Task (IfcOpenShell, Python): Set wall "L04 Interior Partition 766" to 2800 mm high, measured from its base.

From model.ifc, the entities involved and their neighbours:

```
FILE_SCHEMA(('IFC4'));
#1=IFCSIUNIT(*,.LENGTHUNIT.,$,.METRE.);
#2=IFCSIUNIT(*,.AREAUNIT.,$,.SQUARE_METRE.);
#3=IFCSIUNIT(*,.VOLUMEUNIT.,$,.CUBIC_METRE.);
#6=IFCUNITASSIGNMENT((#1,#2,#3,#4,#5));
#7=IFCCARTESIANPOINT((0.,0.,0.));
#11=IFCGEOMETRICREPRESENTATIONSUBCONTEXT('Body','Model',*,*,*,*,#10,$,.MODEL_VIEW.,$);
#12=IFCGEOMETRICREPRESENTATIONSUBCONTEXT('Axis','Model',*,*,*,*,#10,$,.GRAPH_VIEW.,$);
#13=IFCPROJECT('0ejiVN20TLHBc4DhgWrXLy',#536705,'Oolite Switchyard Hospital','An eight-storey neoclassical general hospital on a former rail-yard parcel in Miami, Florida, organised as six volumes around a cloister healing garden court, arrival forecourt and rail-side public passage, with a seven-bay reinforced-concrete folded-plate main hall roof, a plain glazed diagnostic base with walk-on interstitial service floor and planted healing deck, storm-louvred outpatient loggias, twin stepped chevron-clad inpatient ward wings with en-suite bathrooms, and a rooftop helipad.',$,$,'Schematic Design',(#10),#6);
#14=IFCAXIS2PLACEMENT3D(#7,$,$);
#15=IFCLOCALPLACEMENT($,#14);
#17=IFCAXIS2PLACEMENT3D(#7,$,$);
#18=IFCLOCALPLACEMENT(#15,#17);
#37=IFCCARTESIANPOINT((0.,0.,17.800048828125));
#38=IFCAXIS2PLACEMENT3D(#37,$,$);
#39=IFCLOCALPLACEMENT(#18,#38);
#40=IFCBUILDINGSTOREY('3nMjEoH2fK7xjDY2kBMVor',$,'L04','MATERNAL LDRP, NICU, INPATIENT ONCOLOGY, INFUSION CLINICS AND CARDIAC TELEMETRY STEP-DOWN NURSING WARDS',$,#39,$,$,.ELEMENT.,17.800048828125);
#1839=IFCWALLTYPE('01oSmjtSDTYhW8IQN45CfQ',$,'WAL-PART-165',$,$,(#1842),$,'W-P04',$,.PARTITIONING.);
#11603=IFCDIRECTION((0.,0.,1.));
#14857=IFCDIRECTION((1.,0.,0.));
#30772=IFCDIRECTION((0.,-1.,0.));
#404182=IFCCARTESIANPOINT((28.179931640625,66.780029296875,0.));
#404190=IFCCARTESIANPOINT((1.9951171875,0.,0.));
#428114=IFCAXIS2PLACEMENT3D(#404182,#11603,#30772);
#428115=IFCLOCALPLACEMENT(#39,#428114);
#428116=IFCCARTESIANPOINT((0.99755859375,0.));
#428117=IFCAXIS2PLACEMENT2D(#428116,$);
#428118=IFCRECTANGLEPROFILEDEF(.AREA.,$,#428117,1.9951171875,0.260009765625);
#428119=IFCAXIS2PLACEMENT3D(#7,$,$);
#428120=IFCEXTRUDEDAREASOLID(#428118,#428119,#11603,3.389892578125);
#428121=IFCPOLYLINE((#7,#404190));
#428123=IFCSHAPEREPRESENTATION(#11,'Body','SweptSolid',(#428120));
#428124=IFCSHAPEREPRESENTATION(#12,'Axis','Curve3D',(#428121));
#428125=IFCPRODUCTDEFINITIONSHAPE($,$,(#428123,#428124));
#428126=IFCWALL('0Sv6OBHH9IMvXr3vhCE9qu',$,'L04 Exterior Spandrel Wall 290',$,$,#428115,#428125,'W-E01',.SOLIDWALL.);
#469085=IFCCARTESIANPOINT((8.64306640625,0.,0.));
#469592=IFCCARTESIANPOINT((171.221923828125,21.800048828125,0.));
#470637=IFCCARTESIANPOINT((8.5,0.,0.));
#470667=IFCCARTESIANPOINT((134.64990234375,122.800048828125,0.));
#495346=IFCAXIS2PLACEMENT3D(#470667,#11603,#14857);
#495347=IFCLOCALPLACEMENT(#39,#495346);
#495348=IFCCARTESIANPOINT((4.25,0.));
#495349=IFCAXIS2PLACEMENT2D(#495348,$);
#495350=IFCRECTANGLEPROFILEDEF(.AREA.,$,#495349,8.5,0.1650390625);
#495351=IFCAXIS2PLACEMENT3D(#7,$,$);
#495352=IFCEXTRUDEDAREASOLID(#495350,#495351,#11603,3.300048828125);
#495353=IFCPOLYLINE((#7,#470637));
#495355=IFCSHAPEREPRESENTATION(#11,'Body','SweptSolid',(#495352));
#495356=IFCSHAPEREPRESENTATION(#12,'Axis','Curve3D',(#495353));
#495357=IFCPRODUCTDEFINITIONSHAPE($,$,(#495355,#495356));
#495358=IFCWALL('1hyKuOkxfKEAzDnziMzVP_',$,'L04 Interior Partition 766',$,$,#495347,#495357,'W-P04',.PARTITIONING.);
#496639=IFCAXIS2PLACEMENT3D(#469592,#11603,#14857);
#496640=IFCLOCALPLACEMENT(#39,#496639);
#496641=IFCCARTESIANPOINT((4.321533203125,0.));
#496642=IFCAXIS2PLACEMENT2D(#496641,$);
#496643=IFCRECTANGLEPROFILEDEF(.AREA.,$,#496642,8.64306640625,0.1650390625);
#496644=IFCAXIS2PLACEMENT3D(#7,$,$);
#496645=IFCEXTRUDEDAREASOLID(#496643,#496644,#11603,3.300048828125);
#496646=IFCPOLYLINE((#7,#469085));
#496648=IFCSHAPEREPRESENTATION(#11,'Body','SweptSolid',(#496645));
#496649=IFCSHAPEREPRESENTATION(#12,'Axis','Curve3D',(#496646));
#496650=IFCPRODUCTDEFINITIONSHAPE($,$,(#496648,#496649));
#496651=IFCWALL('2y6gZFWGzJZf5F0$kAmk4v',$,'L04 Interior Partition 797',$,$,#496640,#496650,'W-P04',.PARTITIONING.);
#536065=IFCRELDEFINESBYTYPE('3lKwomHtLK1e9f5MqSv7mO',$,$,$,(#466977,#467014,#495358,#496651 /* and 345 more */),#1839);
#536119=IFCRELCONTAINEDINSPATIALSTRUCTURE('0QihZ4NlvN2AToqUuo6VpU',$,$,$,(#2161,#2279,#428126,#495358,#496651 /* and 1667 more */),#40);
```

```python
import ifcopenshell
import ifcopenshell.geom
import ifcopenshell.util.representation
import ifcopenshell.util.shape
import ifcopenshell.util.unit

model = ifcopenshell.open("model.ifc")
unit_scale = ifcopenshell.util.unit.calculate_unit_scale(model)
settings = ifcopenshell.geom.settings()


def volume(element):
    """Net volume in cubic metres, openings subtracted."""
    shape = ifcopenshell.geom.create_shape(settings, element)
    return ifcopenshell.util.shape.get_volume(shape.geometry)


wall = model.by_id(495358)
before = volume(wall)

body = ifcopenshell.util.representation.get_representation(wall, "Model", "Body")
solid = body.Items[0]
old_height = solid.Depth
solid.Depth = 2.8 / unit_scale
after = volume(wall)

print(f"height {old_height:g} -> {solid.Depth:g}, volume {before:.3f} -> {after:.3f} m3")

model.write("model_updated.ifc")
```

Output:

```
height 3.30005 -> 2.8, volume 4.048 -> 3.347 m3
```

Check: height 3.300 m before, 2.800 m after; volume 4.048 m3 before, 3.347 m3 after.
